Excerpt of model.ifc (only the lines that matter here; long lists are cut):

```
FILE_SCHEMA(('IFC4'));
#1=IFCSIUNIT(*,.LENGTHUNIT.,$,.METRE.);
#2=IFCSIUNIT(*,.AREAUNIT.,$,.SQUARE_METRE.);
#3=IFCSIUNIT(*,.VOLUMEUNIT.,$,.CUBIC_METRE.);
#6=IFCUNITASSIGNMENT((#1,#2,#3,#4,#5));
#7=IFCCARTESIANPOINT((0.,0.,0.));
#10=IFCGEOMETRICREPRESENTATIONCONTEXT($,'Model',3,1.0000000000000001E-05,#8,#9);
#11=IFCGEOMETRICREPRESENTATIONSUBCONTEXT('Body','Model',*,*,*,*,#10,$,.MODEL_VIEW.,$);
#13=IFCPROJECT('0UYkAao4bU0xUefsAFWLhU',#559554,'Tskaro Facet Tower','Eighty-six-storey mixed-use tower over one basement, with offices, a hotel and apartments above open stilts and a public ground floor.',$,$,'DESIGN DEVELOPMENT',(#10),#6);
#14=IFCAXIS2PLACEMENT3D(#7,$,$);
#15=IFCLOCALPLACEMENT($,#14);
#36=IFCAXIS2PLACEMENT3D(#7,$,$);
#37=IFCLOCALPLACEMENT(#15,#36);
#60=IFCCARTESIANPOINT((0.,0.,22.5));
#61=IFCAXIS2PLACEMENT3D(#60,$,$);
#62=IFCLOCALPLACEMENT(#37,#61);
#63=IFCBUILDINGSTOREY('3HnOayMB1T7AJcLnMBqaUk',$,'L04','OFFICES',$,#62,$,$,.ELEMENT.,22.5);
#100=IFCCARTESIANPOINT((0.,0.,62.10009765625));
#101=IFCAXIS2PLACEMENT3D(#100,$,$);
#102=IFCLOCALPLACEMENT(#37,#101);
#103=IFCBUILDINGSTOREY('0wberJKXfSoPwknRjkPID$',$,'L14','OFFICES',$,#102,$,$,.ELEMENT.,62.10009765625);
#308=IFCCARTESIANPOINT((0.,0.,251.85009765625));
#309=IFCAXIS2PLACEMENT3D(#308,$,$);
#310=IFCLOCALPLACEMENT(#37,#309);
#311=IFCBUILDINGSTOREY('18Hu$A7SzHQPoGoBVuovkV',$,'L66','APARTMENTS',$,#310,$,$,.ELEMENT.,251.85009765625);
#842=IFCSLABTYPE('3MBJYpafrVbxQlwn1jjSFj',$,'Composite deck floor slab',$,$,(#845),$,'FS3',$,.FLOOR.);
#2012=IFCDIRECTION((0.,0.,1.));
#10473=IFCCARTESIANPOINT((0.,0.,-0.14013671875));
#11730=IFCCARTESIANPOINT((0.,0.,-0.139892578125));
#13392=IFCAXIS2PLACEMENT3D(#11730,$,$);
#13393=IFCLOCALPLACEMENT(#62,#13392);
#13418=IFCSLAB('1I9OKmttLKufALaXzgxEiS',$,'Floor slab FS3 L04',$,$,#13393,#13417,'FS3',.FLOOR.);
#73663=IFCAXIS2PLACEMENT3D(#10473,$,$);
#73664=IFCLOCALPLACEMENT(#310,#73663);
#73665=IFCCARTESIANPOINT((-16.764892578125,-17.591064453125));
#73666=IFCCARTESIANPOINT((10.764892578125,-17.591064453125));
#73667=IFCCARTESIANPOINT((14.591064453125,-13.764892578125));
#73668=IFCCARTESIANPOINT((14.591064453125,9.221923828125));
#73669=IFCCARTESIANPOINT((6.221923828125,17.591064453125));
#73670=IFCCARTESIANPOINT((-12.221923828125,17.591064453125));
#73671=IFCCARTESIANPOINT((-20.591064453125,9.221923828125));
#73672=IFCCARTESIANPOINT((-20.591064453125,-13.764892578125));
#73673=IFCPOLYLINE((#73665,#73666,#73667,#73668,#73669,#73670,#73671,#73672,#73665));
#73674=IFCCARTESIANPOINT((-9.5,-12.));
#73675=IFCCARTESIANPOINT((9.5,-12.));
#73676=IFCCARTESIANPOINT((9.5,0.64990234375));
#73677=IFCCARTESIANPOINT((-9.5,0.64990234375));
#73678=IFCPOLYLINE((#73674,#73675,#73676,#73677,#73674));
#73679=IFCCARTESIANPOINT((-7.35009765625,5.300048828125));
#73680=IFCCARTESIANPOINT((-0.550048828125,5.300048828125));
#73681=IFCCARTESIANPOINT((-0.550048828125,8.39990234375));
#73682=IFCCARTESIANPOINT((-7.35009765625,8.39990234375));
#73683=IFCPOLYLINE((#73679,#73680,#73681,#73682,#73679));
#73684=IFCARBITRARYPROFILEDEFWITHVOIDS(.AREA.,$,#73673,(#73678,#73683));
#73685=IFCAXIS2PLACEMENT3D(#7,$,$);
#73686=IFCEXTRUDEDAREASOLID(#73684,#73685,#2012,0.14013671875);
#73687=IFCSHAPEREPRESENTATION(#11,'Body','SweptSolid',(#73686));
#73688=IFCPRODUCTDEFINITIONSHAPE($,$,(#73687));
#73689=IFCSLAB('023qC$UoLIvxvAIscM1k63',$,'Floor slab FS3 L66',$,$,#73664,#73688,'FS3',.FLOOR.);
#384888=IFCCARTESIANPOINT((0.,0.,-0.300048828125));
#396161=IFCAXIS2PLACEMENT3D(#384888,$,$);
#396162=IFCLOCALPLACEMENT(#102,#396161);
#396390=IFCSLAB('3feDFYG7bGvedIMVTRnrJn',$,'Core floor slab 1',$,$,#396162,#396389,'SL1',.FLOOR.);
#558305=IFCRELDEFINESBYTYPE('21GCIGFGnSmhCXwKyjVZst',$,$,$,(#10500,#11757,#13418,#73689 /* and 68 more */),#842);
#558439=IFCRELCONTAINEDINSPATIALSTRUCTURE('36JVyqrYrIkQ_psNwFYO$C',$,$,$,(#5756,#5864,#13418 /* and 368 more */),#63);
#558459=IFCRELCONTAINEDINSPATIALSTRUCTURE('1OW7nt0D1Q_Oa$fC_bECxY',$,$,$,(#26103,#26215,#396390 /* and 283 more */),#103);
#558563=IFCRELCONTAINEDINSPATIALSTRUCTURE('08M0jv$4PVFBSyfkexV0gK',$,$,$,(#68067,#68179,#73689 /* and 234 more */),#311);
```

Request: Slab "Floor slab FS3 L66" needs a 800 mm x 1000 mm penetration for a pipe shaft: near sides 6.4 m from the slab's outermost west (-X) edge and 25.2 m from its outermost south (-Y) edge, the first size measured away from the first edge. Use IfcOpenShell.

```python
import numpy as np
import ifcopenshell
import ifcopenshell.api.feature
import ifcopenshell.api.geometry
import ifcopenshell.api.root
import ifcopenshell.geom
import ifcopenshell.util.placement
import ifcopenshell.util.representation
import ifcopenshell.util.shape
import ifcopenshell.util.unit

model = ifcopenshell.open("model.ifc")
unit_scale = ifcopenshell.util.unit.calculate_unit_scale(model)
settings = ifcopenshell.geom.settings()


def volume(element):
    """Net volume in cubic metres, openings subtracted."""
    shape = ifcopenshell.geom.create_shape(settings, element)
    return ifcopenshell.util.shape.get_volume(shape.geometry)


slab = model.by_guid("023qC$UoLIvxvAIscM1k63")
before = volume(slab)

# Extent in the slab's own axes, in metres. The edges named are its -X and -Y sides.
slab_shape = ifcopenshell.geom.create_shape(settings, slab)
vertices = ifcopenshell.util.shape.get_vertices(slab_shape.geometry)
x_min, y_min, bottom = vertices.min(axis=0)
top = vertices[:, 2].max()

opening = ifcopenshell.api.root.create_entity(model, ifc_class="IfcOpeningElement", name="Pipe shaft opening", predefined_type="OPENING")
context = ifcopenshell.util.representation.get_context(model, "Model", "Body", "MODEL_VIEW")
width, depth = 0.8, 1
outline = [(0.0, 0.0), (width, 0.0), (width, depth), (0.0, depth), (0.0, 0.0)]
# Overshoot both faces by 50 mm so the cut is clean.
shape = ifcopenshell.api.geometry.add_slab_representation(
    model, context=context, depth=top - bottom + 0.1, polyline=outline
)
ifcopenshell.api.geometry.assign_representation(model, product=opening, representation=shape)

matrix = ifcopenshell.util.placement.get_local_placement(slab.ObjectPlacement)
matrix[:, 3] = matrix @ np.append(np.array([x_min + 6.4, y_min + 25.2, bottom - 0.05]) / unit_scale, 1.0)
ifcopenshell.api.geometry.edit_object_placement(model, product=opening, matrix=matrix, is_si=False)
ifcopenshell.api.feature.add_feature(model, feature=opening, element=slab)

after = volume(slab)

print(f"slab volume {before:.3f} -> {after:.3f} m3")

model.write("model_rev.ifc")
```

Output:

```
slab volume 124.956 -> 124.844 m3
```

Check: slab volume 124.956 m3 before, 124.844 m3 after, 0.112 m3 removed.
